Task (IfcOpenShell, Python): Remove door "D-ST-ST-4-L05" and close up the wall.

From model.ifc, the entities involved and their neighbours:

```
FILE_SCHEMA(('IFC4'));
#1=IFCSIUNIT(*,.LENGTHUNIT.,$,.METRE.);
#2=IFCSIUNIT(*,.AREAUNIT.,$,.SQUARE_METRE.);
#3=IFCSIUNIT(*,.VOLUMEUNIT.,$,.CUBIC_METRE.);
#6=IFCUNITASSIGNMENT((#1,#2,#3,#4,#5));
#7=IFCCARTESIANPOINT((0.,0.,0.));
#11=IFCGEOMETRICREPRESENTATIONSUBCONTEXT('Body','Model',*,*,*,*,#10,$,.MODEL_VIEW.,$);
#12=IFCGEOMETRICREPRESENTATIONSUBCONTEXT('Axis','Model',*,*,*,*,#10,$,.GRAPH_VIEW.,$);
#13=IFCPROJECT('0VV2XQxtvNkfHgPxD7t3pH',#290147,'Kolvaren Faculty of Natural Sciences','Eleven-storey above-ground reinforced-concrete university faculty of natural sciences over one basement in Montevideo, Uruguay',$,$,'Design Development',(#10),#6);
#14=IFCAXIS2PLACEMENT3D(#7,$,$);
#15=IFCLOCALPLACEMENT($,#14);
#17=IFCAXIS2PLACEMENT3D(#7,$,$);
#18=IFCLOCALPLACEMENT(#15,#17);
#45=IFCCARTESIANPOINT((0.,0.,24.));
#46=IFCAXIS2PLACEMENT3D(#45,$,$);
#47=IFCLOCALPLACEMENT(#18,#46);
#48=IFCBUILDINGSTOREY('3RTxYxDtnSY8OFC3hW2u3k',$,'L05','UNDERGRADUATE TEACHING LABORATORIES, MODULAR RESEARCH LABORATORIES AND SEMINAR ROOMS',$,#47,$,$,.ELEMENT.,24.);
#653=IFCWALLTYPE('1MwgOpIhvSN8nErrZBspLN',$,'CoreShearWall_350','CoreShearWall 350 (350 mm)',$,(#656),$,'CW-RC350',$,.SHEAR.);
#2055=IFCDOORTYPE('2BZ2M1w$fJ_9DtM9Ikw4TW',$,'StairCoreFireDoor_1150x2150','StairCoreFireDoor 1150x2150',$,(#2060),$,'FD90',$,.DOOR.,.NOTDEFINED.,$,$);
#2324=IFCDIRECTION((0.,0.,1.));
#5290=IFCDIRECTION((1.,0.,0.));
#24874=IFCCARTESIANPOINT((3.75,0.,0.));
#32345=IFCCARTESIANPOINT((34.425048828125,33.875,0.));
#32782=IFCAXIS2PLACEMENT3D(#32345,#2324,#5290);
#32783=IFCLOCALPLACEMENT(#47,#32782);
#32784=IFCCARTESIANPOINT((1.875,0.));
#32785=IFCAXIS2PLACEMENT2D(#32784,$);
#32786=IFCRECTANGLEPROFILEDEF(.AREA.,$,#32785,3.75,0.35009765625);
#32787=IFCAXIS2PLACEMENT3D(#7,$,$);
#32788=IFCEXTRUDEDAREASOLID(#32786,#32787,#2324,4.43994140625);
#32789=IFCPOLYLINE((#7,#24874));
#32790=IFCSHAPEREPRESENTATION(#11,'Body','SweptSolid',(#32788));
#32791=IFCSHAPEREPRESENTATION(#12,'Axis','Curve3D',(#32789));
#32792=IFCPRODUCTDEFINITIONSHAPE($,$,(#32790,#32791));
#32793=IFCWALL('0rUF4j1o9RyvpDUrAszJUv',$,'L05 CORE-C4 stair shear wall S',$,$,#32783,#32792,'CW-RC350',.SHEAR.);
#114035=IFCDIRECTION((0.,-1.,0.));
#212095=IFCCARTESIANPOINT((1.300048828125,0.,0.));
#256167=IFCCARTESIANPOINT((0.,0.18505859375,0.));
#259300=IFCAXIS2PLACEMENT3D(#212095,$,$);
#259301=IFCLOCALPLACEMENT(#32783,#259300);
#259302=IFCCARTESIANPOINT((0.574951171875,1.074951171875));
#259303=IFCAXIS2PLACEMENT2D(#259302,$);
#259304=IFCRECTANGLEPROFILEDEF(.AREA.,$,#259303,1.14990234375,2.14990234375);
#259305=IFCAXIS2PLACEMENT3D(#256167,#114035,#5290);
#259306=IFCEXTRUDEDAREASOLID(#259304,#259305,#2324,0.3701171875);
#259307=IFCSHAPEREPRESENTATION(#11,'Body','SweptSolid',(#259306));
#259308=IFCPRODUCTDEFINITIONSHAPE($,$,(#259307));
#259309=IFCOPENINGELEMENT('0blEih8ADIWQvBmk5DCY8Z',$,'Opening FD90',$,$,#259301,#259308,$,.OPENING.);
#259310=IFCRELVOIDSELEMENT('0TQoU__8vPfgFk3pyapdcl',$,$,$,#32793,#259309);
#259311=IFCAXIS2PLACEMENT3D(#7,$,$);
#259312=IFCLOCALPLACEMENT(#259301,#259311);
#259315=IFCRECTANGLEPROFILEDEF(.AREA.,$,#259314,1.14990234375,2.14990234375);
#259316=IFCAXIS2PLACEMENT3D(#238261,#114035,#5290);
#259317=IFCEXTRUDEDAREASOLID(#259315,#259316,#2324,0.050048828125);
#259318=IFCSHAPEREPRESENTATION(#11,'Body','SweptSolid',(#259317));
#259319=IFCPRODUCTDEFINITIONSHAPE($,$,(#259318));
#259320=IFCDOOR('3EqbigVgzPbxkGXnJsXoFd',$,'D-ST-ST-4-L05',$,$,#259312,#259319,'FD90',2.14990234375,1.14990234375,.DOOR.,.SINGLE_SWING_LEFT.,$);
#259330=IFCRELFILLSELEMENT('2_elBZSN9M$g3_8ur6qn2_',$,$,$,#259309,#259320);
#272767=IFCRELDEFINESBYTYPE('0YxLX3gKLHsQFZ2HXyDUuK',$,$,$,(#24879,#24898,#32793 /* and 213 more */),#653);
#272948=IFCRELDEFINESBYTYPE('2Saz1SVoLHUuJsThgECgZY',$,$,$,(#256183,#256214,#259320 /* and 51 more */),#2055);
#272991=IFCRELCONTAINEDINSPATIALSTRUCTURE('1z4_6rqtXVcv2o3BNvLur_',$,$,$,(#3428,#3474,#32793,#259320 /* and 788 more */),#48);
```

```python
import ifcopenshell
import ifcopenshell.api.feature
import ifcopenshell.api.root
import ifcopenshell.geom
import ifcopenshell.util.shape

model = ifcopenshell.open("model.ifc")
settings = ifcopenshell.geom.settings()


def volume(element):
    """Net volume in cubic metres, openings subtracted."""
    shape = ifcopenshell.geom.create_shape(settings, element)
    return ifcopenshell.util.shape.get_volume(shape.geometry)


door = model.by_guid("3EqbigVgzPbxkGXnJsXoFd")
opening = door.FillsVoids[0].RelatingOpeningElement
wall = opening.VoidsElements[0].RelatingBuildingElement
before = volume(wall)

ifcopenshell.api.root.remove_product(model, product=door)
ifcopenshell.api.feature.remove_feature(model, feature=opening)

after = volume(wall)

print(f"wall volume {before:.3f} -> {after:.3f} m3")

model.write("model-out.ifc")
```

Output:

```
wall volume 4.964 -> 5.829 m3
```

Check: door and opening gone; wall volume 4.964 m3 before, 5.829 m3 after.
